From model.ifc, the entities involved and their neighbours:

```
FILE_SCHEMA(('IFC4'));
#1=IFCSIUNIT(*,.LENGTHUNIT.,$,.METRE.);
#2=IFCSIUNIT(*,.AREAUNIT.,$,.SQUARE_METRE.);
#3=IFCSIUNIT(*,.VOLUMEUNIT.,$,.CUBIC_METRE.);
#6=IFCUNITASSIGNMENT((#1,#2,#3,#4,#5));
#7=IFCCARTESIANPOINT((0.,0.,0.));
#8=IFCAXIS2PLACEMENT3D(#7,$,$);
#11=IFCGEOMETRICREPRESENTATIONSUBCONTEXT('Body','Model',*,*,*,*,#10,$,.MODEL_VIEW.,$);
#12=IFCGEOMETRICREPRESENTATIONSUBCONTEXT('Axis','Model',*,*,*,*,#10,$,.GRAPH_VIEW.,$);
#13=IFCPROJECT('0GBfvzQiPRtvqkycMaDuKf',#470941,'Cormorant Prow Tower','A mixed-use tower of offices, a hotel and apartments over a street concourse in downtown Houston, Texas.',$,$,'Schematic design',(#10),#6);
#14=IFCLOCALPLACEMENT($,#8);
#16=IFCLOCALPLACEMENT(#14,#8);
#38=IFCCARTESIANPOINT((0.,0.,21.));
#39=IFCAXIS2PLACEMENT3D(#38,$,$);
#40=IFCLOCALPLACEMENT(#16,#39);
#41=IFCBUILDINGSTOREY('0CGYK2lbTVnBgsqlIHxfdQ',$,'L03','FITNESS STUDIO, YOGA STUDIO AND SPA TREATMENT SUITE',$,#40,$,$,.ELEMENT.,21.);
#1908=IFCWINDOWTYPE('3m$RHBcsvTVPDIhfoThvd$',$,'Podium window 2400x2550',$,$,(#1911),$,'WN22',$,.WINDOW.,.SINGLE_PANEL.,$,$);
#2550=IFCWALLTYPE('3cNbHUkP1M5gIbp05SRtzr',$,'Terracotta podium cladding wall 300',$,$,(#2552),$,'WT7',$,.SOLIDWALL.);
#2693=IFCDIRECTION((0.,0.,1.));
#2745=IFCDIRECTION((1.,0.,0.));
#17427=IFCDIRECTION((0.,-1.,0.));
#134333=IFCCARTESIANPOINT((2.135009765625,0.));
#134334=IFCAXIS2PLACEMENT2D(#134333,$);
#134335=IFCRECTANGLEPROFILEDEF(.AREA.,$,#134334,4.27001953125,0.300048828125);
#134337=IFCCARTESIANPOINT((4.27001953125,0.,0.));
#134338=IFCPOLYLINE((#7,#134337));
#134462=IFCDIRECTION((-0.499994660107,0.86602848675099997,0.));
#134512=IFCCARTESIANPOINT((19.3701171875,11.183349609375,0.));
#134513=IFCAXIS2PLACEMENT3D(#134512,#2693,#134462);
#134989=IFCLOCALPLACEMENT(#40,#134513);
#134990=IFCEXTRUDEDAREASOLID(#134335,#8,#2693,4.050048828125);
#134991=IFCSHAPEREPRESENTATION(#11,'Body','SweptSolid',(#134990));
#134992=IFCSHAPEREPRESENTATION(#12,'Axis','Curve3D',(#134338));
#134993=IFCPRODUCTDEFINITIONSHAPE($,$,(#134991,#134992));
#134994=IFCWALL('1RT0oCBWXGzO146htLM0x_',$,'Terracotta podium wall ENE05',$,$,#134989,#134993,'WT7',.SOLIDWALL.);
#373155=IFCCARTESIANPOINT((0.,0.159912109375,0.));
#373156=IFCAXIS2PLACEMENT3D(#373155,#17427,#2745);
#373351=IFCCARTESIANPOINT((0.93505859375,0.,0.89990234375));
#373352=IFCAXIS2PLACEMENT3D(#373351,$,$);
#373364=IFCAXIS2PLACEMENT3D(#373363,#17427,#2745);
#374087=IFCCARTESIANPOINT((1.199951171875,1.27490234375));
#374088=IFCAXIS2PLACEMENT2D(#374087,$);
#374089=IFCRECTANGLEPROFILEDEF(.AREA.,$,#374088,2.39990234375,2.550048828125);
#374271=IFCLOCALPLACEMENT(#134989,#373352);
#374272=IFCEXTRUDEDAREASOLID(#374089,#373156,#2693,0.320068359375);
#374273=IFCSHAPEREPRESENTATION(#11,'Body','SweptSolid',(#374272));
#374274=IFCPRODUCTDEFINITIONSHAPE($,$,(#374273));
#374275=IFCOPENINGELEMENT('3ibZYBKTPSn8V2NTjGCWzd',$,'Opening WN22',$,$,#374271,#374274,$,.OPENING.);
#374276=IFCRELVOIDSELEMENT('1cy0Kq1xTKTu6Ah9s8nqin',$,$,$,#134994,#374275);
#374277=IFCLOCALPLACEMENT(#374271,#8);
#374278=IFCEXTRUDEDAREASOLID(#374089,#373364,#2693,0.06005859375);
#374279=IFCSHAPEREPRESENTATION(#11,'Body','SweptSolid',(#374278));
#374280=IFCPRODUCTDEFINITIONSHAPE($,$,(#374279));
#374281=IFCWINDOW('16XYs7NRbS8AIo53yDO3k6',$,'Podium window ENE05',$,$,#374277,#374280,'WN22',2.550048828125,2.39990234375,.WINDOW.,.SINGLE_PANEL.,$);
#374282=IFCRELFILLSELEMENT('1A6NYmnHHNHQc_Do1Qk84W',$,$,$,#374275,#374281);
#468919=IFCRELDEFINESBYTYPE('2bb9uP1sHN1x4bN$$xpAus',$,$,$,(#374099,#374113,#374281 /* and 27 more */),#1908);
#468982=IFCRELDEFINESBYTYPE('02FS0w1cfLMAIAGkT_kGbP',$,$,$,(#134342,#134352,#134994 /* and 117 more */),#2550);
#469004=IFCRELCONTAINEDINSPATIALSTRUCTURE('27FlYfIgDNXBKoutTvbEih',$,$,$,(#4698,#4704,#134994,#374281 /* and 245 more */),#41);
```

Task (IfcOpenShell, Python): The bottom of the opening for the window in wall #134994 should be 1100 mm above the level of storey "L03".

```python
import numpy as np
import ifcopenshell
import ifcopenshell.api.geometry
import ifcopenshell.geom
import ifcopenshell.util.element
import ifcopenshell.util.placement
import ifcopenshell.util.shape
import ifcopenshell.util.unit

model = ifcopenshell.open("model.ifc")
unit_scale = ifcopenshell.util.unit.calculate_unit_scale(model)

window = model.by_guid("16XYs7NRbS8AIo53yDO3k6")
opening = window.FillsVoids[0].RelatingOpeningElement
storey = ifcopenshell.util.element.get_container(window, ifc_class="IfcBuildingStorey")
level = ifcopenshell.util.placement.get_local_placement(storey.ObjectPlacement)[2, 3]

# The opening's origin need not be at the sill, so measure its lowest point.
shape = ifcopenshell.geom.create_shape(ifcopenshell.geom.settings(), opening)
bottom = ifcopenshell.util.shape.get_shape_bottom_elevation(shape, shape.geometry) / unit_scale
dz = level + 1.1 - bottom

shift = np.array([0.0, 0.0, dz])
# The window is placed relative to its opening, so it follows when the opening moves.
matrix = ifcopenshell.util.placement.get_local_placement(opening.ObjectPlacement)
matrix[:3, 3] += shift
ifcopenshell.api.geometry.edit_object_placement(
    model, product=opening, matrix=matrix, is_si=False, should_transform_children=True
)

print(f"moved by {dz * unit_scale:+.3f} m")

model.write("model-out.ifc")
```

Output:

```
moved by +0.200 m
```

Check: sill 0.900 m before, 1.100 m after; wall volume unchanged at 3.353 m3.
